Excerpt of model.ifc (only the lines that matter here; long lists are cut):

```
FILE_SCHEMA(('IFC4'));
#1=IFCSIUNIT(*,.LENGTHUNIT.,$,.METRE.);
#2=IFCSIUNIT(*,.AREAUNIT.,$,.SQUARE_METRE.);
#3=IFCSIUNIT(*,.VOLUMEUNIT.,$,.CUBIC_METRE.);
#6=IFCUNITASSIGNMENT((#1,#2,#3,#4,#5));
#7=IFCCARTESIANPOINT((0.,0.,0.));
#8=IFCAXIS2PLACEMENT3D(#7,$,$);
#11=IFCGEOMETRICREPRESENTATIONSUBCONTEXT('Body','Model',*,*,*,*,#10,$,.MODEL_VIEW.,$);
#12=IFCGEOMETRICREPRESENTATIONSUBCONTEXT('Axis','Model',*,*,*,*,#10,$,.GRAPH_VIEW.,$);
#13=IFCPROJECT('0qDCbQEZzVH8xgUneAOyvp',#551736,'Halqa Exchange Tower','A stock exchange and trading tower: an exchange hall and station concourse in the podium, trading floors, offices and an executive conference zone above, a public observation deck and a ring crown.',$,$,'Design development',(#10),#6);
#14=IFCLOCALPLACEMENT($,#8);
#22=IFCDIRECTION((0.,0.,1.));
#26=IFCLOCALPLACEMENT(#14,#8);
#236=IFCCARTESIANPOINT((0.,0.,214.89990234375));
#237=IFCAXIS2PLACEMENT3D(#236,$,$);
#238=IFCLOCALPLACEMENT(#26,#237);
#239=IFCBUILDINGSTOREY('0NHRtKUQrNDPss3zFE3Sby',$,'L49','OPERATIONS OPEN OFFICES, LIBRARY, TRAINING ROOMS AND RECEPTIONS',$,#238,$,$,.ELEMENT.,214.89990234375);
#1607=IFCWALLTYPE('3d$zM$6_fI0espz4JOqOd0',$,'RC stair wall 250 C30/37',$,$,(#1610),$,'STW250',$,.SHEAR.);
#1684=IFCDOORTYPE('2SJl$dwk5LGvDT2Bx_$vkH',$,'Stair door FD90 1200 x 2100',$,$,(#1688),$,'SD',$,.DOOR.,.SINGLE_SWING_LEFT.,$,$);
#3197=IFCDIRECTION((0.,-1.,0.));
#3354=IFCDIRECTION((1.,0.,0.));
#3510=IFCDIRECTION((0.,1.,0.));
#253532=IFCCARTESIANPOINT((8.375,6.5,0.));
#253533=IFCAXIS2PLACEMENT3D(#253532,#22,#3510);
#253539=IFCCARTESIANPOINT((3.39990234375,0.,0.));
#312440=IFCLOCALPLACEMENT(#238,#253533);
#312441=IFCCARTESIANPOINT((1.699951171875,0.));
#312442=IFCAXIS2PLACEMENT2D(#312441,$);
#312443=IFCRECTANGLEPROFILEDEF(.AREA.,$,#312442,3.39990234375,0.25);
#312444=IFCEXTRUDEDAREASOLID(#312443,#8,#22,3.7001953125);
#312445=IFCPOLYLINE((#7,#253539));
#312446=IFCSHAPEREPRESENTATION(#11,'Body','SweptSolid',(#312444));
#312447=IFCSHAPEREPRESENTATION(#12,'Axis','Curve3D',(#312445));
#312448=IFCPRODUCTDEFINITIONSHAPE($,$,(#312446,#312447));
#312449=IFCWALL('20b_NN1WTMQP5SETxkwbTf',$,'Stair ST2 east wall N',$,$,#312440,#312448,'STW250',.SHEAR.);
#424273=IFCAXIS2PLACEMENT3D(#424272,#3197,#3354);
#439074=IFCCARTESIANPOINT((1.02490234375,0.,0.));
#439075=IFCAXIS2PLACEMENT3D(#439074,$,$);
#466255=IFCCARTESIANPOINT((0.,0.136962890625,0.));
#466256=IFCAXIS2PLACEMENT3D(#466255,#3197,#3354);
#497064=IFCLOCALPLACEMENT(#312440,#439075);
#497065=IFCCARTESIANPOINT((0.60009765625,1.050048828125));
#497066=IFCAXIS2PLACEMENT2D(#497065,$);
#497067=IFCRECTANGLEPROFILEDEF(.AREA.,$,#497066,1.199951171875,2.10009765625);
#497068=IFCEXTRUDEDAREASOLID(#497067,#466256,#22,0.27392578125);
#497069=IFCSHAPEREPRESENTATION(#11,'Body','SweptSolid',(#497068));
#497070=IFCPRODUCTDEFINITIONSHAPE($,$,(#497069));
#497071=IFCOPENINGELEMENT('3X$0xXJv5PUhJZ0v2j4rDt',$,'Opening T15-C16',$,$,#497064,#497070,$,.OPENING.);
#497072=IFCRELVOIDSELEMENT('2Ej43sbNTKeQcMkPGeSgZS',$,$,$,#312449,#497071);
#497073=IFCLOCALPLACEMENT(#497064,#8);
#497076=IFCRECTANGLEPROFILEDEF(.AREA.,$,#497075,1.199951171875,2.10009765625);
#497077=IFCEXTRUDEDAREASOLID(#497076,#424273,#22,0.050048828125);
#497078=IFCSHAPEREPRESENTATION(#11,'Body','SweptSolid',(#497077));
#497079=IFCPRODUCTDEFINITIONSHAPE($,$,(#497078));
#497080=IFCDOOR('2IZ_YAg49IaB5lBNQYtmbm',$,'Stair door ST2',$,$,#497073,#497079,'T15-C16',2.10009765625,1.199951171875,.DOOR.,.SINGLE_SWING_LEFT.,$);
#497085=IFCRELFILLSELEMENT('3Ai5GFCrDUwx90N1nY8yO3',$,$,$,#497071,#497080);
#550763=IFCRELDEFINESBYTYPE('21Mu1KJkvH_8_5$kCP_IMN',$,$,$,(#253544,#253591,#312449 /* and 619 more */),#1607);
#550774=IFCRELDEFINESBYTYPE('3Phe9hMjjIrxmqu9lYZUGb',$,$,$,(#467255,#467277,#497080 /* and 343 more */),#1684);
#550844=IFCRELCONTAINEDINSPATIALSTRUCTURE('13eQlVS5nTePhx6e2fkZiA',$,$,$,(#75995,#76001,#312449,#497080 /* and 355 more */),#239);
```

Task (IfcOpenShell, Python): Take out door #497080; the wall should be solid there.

```python
import ifcopenshell
import ifcopenshell.api.feature
import ifcopenshell.api.root
import ifcopenshell.geom
import ifcopenshell.util.shape

model = ifcopenshell.open("model.ifc")
settings = ifcopenshell.geom.settings()


def volume(element):
    """Net volume in cubic metres, openings subtracted."""
    shape = ifcopenshell.geom.create_shape(settings, element)
    return ifcopenshell.util.shape.get_volume(shape.geometry)


door = model.by_guid("2IZ_YAg49IaB5lBNQYtmbm")
opening = door.FillsVoids[0].RelatingOpeningElement
wall = opening.VoidsElements[0].RelatingBuildingElement
before = volume(wall)

ifcopenshell.api.root.remove_product(model, product=door)
ifcopenshell.api.feature.remove_feature(model, feature=opening)

after = volume(wall)

print(f"wall volume {before:.3f} -> {after:.3f} m3")

model.write("model_v2.ifc")
```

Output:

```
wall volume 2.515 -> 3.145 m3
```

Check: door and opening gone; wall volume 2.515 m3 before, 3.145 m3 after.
